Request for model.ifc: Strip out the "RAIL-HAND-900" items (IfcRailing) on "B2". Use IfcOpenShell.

First a look at what the model holds.

```python
import ifcopenshell
import ifcopenshell.util.element

model = ifcopenshell.open("model.ifc")
print(model.schema)
storey = next(s for s in model.by_type("IfcBuildingStorey") if s.Name == "B2")
railings = [e for e in ifcopenshell.util.element.get_decomposition(storey) if e.is_a("IfcRailing")]
seen = {}
for e in railings:
    element_type = ifcopenshell.util.element.get_type(e)
    name = element_type.Name if element_type not in (None, e) else None
    seen[name] = seen.get(name, 0) + 1
for name, count in sorted(seen.items(), key=str):
    print(count, "x", name)
```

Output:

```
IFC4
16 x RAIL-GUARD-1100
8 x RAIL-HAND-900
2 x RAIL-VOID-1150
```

```python
import ifcopenshell
import ifcopenshell.api.root
import ifcopenshell.util.element

model = ifcopenshell.open("model.ifc")

storey = next(s for s in model.by_type("IfcBuildingStorey") if s.Name == "B2")
railings = [e for e in ifcopenshell.util.element.get_decomposition(storey) if e.is_a("IfcRailing")]
targets = [e for e in railings if (t := ifcopenshell.util.element.get_type(e)) not in (None, e) and t.Name == "RAIL-HAND-900"]

for e in targets:
    ifcopenshell.api.root.remove_product(model, product=e)
print(len(targets), "removed")

model.write("model_updated.ifc")
```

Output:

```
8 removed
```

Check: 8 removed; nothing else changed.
